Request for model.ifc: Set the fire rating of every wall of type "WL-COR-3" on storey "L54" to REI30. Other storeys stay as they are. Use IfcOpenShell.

First a look at what the model holds.

```python
import ifcopenshell
import ifcopenshell.util.element

model = ifcopenshell.open("model.ifc")
print(model.schema)
storey = next(s for s in model.by_type("IfcBuildingStorey") if s.Name == "L54")
walls = [e for e in ifcopenshell.util.element.get_decomposition(storey) if e.is_a("IfcWall")]
seen = {}
for e in walls:
    element_type = ifcopenshell.util.element.get_type(e)
    key = (element_type.Name if element_type != e and element_type else None, ifcopenshell.util.element.get_pset(e, "Pset_WallCommon", "FireRating"))
    seen[key] = seen.get(key, 0) + 1
for (name, value), count in sorted(seen.items(), key=str):
    print(count, "x", name, "|", value)
```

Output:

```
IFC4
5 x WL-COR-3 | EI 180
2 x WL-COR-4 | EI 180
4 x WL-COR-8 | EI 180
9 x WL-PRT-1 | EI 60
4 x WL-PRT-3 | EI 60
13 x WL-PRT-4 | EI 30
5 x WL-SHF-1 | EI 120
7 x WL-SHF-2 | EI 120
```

```python
import ifcopenshell
import ifcopenshell.api.pset
import ifcopenshell.util.element

model = ifcopenshell.open("model.ifc")

storey = next(s for s in model.by_type("IfcBuildingStorey") if s.Name == "L54")
walls = [e for e in ifcopenshell.util.element.get_decomposition(storey) if e.is_a("IfcWall")]

count = 0
for e in walls:
    element_type = ifcopenshell.util.element.get_type(e)
    if element_type in (None, e) or element_type.Name != "WL-COR-3":
        continue
    # add_pset returns the element's existing set when there is one.
    pset = ifcopenshell.api.pset.add_pset(model, product=e, name="Pset_WallCommon")
    ifcopenshell.api.pset.edit_pset(model, pset=pset, properties={"FireRating": "REI30"})
    count += 1

print(count, "walls updated")

model.write("model_rev.ifc")
```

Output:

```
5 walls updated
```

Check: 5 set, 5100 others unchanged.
